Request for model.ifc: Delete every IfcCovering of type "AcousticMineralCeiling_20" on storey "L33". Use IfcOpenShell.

First a look at what the model holds.

```python
import ifcopenshell
import ifcopenshell.util.element

model = ifcopenshell.open("model.ifc")
print(model.schema)
storey = next(s for s in model.by_type("IfcBuildingStorey") if s.Name == "L33")
coverings = [e for e in ifcopenshell.util.element.get_decomposition(storey) if e.is_a("IfcCovering")]
seen = {}
for e in coverings:
    element_type = ifcopenshell.util.element.get_type(e)
    name = element_type.Name if element_type not in (None, e) else None
    seen[name] = seen.get(name, 0) + 1
for name, count in sorted(seen.items(), key=str):
    print(count, "x", name)
```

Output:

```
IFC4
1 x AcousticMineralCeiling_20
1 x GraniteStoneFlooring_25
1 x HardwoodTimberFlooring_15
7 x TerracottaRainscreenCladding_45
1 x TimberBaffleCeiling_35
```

```python
import ifcopenshell
import ifcopenshell.api.root
import ifcopenshell.util.element

model = ifcopenshell.open("model.ifc")

storey = next(s for s in model.by_type("IfcBuildingStorey") if s.Name == "L33")
coverings = [e for e in ifcopenshell.util.element.get_decomposition(storey) if e.is_a("IfcCovering")]
targets = [e for e in coverings if (t := ifcopenshell.util.element.get_type(e)) not in (None, e) and t.Name == "AcousticMineralCeiling_20"]

for e in targets:
    ifcopenshell.api.root.remove_product(model, product=e)
print(len(targets), "removed")

model.write("model_updated.ifc")
```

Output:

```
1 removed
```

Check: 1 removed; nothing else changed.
